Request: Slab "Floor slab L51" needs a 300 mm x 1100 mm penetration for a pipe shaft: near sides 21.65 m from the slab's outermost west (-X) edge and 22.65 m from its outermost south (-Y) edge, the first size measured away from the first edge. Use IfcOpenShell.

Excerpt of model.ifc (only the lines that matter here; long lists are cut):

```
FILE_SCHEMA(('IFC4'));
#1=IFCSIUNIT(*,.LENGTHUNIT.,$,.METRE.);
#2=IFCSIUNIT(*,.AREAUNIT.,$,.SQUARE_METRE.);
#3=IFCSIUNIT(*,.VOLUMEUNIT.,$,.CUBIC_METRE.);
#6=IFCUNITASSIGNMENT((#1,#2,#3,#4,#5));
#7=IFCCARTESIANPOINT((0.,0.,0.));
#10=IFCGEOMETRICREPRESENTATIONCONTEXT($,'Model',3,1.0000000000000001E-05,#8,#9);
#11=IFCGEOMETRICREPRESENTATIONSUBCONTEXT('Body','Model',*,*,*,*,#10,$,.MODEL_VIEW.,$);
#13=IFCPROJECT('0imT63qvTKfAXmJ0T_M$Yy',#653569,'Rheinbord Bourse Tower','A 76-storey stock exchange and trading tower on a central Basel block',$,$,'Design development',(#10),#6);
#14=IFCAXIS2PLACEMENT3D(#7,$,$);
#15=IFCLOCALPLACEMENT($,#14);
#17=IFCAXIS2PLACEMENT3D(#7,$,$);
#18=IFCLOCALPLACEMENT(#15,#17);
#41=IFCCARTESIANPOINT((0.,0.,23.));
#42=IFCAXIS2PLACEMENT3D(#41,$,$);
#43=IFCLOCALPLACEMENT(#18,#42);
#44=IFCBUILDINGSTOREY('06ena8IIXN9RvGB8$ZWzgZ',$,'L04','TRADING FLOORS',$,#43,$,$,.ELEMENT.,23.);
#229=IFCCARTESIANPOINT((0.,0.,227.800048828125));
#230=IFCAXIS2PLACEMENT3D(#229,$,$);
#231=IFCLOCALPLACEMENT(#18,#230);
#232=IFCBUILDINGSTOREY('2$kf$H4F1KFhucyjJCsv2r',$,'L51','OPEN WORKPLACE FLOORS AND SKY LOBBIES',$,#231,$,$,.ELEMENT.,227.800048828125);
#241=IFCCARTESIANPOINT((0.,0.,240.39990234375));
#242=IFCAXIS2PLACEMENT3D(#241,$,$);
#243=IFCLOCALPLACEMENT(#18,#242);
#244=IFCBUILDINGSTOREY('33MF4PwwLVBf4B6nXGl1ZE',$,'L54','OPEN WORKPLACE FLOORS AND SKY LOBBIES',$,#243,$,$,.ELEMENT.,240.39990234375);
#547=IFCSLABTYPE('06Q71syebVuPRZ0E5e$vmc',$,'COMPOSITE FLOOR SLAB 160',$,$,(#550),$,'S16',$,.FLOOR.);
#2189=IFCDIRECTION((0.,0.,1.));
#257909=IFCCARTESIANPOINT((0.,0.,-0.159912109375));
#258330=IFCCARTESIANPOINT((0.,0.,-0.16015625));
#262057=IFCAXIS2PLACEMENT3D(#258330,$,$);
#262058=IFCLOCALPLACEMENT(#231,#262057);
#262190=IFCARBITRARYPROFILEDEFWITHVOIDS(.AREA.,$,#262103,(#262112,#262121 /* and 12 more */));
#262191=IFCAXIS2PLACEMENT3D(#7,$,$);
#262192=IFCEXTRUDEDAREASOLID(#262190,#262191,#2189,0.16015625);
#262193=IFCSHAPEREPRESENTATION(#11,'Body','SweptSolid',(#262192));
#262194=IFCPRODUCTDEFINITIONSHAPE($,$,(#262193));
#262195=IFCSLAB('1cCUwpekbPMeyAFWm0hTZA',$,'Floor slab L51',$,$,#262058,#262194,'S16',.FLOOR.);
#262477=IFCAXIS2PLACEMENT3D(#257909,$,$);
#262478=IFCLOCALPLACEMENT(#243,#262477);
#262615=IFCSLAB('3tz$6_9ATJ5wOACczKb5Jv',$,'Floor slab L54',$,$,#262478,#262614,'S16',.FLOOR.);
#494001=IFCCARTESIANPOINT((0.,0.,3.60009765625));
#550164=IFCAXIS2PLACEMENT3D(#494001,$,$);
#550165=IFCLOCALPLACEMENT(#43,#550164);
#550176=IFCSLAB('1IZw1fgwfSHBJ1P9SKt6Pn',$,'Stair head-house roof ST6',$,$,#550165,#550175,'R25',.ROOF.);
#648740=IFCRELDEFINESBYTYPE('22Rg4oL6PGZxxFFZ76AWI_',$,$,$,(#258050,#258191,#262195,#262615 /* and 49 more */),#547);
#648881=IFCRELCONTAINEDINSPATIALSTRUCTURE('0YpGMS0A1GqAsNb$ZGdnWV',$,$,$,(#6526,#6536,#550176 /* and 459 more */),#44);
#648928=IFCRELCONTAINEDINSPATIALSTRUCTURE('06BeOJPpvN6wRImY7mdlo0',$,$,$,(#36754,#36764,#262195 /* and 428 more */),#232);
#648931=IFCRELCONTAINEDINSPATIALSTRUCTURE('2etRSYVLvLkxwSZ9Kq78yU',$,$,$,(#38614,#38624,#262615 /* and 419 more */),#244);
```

```python
import numpy as np
import ifcopenshell
import ifcopenshell.api.feature
import ifcopenshell.api.geometry
import ifcopenshell.api.root
import ifcopenshell.geom
import ifcopenshell.util.placement
import ifcopenshell.util.representation
import ifcopenshell.util.shape
import ifcopenshell.util.unit

model = ifcopenshell.open("model.ifc")
unit_scale = ifcopenshell.util.unit.calculate_unit_scale(model)
settings = ifcopenshell.geom.settings()


def volume(element):
    """Net volume in cubic metres, openings subtracted."""
    shape = ifcopenshell.geom.create_shape(settings, element)
    return ifcopenshell.util.shape.get_volume(shape.geometry)


slab = model.by_guid("1cCUwpekbPMeyAFWm0hTZA")
before = volume(slab)

# Extent in the slab's own axes, in metres. The edges named are its -X and -Y sides.
slab_shape = ifcopenshell.geom.create_shape(settings, slab)
vertices = ifcopenshell.util.shape.get_vertices(slab_shape.geometry)
x_min, y_min, bottom = vertices.min(axis=0)
top = vertices[:, 2].max()

opening = ifcopenshell.api.root.create_entity(model, ifc_class="IfcOpeningElement", name="Pipe shaft opening", predefined_type="OPENING")
context = ifcopenshell.util.representation.get_context(model, "Model", "Body", "MODEL_VIEW")
width, depth = 0.3, 1.1
outline = [(0.0, 0.0), (width, 0.0), (width, depth), (0.0, depth), (0.0, 0.0)]
# Overshoot both faces by 50 mm so the cut is clean.
shape = ifcopenshell.api.geometry.add_slab_representation(
    model, context=context, depth=top - bottom + 0.1, polyline=outline
)
ifcopenshell.api.geometry.assign_representation(model, product=opening, representation=shape)

matrix = ifcopenshell.util.placement.get_local_placement(slab.ObjectPlacement)
matrix[:, 3] = matrix @ np.append(np.array([x_min + 21.65, y_min + 22.65, bottom - 0.05]) / unit_scale, 1.0)
ifcopenshell.api.geometry.edit_object_placement(model, product=opening, matrix=matrix, is_si=False)
ifcopenshell.api.feature.add_feature(model, feature=opening, element=slab)

after = volume(slab)

print(f"slab volume {before:.3f} -> {after:.3f} m3")

model.write("model_v2.ifc")
```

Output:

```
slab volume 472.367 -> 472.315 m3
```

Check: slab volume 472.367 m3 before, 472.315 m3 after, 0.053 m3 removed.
